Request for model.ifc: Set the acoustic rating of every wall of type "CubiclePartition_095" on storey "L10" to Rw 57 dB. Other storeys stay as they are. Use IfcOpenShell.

First a look at what the model holds.

```python
import ifcopenshell
import ifcopenshell.util.element

model = ifcopenshell.open("model.ifc")
print(model.schema)
storey = next(s for s in model.by_type("IfcBuildingStorey") if s.Name == "L10")
walls = [e for e in ifcopenshell.util.element.get_decomposition(storey) if e.is_a("IfcWall")]
seen = {}
for e in walls:
    element_type = ifcopenshell.util.element.get_type(e)
    key = (element_type.Name if element_type != e and element_type else None, ifcopenshell.util.element.get_pset(e, "Pset_WallCommon", "AcousticRating"))
    seen[key] = seen.get(key, 0) + 1
for (name, value), count in sorted(seen.items(), key=str):
    print(count, "x", name, "|", value)
```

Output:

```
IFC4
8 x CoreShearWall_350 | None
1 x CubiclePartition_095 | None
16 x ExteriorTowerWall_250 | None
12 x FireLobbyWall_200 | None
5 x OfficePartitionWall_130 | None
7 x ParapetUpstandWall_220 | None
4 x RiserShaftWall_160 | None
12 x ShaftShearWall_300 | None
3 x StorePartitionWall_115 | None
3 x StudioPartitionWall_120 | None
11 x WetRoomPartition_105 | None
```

```python
import ifcopenshell
import ifcopenshell.api.pset
import ifcopenshell.util.element

model = ifcopenshell.open("model.ifc")

storey = next(s for s in model.by_type("IfcBuildingStorey") if s.Name == "L10")
walls = [e for e in ifcopenshell.util.element.get_decomposition(storey) if e.is_a("IfcWall")]

count = 0
for e in walls:
    element_type = ifcopenshell.util.element.get_type(e)
    if element_type in (None, e) or element_type.Name != "CubiclePartition_095":
        continue
    # add_pset returns the element's existing set when there is one.
    pset = ifcopenshell.api.pset.add_pset(model, product=e, name="Pset_WallCommon")
    ifcopenshell.api.pset.edit_pset(model, pset=pset, properties={"AcousticRating": "Rw 57 dB"})
    count += 1

print(count, "walls updated")

model.write("model_updated.ifc")
```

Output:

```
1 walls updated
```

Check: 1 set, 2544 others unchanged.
